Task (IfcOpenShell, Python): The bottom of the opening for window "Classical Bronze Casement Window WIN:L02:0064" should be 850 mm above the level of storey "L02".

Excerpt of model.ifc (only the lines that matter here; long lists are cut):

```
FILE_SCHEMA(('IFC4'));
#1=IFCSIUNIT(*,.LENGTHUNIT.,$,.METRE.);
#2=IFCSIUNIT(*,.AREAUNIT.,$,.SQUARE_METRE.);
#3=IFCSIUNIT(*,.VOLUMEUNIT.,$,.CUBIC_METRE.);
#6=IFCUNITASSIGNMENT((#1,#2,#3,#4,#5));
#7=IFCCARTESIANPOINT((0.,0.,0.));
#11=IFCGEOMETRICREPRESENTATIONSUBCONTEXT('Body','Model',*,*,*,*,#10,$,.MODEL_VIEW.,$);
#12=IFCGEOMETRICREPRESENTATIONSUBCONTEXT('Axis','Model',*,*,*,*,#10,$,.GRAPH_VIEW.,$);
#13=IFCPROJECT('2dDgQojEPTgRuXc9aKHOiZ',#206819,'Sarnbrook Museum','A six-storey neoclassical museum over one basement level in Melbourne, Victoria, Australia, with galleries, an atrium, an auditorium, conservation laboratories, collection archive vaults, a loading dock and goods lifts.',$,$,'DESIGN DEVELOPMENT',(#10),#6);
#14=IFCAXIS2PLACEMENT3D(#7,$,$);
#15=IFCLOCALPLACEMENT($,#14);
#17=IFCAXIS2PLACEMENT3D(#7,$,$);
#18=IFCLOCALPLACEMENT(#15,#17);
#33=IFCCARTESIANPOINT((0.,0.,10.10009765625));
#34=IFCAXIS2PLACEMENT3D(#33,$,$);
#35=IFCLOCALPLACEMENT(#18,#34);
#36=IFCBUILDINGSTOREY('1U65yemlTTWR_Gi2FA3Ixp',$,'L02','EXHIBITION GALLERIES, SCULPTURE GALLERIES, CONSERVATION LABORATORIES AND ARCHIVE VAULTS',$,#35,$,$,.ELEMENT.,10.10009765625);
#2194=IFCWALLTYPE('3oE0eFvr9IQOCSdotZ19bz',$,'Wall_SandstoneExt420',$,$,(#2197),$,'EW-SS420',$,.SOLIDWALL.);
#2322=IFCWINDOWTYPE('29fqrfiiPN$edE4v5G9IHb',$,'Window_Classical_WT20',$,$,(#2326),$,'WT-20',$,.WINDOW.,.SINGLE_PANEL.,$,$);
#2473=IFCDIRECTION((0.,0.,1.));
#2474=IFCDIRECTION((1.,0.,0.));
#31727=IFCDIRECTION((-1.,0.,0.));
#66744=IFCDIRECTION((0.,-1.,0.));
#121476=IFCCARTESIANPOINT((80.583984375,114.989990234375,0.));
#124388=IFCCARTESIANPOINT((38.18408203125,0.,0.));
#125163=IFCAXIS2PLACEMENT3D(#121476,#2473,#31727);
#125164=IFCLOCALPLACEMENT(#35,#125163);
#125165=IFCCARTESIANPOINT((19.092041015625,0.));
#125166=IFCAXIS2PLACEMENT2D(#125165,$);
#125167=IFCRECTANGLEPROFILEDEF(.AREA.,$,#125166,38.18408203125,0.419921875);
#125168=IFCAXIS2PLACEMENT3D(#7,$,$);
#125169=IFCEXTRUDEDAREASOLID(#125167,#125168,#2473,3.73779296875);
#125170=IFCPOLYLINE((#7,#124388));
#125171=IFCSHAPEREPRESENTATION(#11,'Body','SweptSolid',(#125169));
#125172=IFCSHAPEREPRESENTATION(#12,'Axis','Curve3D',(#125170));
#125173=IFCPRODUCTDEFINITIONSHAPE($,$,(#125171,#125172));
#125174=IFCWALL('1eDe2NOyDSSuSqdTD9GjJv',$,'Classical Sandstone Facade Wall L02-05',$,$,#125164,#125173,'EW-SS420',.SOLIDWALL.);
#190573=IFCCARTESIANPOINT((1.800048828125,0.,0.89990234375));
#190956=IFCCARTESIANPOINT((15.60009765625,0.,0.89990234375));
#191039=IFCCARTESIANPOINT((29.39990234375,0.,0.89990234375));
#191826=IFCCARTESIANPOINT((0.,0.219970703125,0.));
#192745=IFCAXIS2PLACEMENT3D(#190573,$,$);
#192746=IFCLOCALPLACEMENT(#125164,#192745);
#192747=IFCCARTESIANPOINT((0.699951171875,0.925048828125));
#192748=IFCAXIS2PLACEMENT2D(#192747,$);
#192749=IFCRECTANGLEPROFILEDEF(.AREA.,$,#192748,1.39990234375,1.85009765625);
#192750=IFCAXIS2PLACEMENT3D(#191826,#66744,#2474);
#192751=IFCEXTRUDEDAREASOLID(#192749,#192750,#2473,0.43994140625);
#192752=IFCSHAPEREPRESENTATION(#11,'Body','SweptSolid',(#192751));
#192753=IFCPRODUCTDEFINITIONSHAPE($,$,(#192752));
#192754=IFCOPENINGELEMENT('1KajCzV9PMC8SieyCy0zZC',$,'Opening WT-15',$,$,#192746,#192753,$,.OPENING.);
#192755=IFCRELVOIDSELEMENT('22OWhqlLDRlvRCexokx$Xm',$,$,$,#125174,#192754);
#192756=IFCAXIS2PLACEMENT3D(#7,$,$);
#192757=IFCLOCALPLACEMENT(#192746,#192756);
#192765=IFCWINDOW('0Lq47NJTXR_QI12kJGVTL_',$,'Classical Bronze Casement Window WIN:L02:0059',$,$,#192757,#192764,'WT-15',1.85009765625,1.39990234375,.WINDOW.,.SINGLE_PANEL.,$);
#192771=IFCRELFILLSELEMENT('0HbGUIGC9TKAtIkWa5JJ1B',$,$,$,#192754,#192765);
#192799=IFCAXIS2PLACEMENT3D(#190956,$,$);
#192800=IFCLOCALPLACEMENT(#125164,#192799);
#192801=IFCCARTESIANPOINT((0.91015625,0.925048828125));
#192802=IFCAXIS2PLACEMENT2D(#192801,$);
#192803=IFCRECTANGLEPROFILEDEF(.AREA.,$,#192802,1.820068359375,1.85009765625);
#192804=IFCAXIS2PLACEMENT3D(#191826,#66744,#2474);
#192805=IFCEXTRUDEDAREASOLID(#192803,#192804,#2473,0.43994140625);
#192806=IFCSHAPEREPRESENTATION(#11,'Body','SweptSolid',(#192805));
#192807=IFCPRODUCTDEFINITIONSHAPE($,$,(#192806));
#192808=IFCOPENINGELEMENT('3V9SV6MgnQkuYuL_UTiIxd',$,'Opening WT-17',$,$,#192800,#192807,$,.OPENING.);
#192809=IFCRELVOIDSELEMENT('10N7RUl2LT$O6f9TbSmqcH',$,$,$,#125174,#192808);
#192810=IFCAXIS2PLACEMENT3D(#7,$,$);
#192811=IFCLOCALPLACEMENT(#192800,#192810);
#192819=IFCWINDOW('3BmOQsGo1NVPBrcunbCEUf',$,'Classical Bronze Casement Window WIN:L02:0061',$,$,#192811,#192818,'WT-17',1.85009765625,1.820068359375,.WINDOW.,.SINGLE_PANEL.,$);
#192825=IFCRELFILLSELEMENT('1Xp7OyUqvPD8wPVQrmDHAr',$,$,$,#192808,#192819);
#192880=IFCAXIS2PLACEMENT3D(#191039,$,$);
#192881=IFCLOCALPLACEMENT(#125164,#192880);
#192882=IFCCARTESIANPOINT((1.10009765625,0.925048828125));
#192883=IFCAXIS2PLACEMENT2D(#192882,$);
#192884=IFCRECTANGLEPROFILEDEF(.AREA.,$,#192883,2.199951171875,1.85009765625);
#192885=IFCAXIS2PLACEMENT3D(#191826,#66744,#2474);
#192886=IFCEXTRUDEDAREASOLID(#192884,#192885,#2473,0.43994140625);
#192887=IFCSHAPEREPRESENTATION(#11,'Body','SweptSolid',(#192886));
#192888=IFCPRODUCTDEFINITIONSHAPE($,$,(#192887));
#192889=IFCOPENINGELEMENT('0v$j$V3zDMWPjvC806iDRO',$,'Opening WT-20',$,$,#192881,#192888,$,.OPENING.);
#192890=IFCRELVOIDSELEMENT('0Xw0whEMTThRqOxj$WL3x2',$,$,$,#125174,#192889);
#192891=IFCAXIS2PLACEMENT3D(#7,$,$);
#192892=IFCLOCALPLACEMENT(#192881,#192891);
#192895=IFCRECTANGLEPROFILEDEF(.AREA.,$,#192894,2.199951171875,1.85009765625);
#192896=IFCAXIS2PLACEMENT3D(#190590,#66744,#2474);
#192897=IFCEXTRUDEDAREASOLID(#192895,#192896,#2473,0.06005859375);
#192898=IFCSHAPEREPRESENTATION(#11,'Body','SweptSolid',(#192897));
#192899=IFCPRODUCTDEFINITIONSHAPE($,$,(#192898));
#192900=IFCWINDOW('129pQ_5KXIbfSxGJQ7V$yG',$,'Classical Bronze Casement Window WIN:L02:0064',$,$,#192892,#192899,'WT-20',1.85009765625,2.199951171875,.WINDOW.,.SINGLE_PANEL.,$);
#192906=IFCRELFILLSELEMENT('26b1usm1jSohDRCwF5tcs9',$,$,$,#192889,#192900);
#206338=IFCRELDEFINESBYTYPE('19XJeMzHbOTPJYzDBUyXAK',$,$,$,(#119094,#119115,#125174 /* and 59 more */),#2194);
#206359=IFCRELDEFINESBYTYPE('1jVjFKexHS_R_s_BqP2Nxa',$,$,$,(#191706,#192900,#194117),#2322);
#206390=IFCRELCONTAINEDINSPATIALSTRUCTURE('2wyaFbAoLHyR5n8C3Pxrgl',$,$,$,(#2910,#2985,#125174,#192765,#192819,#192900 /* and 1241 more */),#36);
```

```python
import numpy as np
import ifcopenshell
import ifcopenshell.api.geometry
import ifcopenshell.geom
import ifcopenshell.util.element
import ifcopenshell.util.placement
import ifcopenshell.util.shape
import ifcopenshell.util.unit

model = ifcopenshell.open("model.ifc")
unit_scale = ifcopenshell.util.unit.calculate_unit_scale(model)

window = model.by_id(192900)
opening = window.FillsVoids[0].RelatingOpeningElement
storey = ifcopenshell.util.element.get_container(window, ifc_class="IfcBuildingStorey")
level = ifcopenshell.util.placement.get_local_placement(storey.ObjectPlacement)[2, 3]

# The opening's origin need not be at the sill, so measure its lowest point.
shape = ifcopenshell.geom.create_shape(ifcopenshell.geom.settings(), opening)
bottom = ifcopenshell.util.shape.get_shape_bottom_elevation(shape, shape.geometry) / unit_scale
dz = level + 0.85 / unit_scale - bottom

shift = np.array([0.0, 0.0, dz])
# The window is placed relative to its opening, so it follows when the opening moves.
matrix = ifcopenshell.util.placement.get_local_placement(opening.ObjectPlacement)
matrix[:3, 3] += shift
ifcopenshell.api.geometry.edit_object_placement(
    model, product=opening, matrix=matrix, is_si=False, should_transform_children=True
)

print(f"moved by {dz * unit_scale:+.3f} m")

model.write("model_rev.ifc")
```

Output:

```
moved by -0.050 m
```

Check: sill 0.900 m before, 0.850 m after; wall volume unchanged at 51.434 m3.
